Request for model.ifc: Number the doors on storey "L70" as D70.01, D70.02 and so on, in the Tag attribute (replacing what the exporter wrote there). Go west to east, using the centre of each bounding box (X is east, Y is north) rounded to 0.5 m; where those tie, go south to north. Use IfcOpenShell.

First a look at what the model holds.

```python
import ifcopenshell
import ifcopenshell.util.element
import ifcopenshell.util.placement

model = ifcopenshell.open("model.ifc")
print(model.schema)
storey = next(s for s in model.by_type("IfcBuildingStorey") if s.Name == "L70")
doors = [e for e in ifcopenshell.util.element.get_decomposition(storey) if e.is_a("IfcDoor")]
for e in sorted(doors, key=lambda e: e.id()):
    origin = ifcopenshell.util.placement.get_local_placement(e.ObjectPlacement)[:3, 3]
    print(e.id(), e.Tag, e.Name, origin.round(2) + 0.0, sep=" | ")
```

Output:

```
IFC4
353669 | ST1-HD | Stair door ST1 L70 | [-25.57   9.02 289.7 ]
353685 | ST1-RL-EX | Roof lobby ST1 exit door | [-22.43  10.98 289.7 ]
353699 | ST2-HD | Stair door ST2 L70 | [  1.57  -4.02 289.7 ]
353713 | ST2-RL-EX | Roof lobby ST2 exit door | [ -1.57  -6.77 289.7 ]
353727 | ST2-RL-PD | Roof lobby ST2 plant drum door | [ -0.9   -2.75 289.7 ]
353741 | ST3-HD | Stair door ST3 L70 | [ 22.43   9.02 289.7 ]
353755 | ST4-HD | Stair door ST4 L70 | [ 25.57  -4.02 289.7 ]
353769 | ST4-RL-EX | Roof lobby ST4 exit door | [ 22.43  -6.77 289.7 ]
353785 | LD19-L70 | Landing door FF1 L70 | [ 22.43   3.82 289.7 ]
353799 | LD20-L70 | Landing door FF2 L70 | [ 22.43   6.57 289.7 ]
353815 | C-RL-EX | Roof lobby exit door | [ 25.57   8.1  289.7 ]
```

```python
import ifcopenshell
import ifcopenshell.geom
import ifcopenshell.util.element
import ifcopenshell.util.shape

model = ifcopenshell.open("model.ifc")
settings = ifcopenshell.geom.settings()
settings.set("use-world-coords", True)


def centre(element):
    shape = ifcopenshell.geom.create_shape(settings, element)
    return ifcopenshell.util.shape.get_bbox_centroid(shape.geometry)


storey = next(s for s in model.by_type("IfcBuildingStorey") if s.Name == "L70")
doors = [e for e in ifcopenshell.util.element.get_decomposition(storey) if e.is_a("IfcDoor")]

# Insertion points can sit at a corner or the storey origin, so sort by the geometry (in metres).
centres = {e: centre(e) for e in doors}
doors.sort(key=lambda e: (round(centres[e][0] / 0.5), centres[e][1]))

for i, e in enumerate(doors, start=1):
    number = f"D70.{i:02d}"
    e.Tag = number
    print(e.id(), number)

model.write("model_v2.ifc")
```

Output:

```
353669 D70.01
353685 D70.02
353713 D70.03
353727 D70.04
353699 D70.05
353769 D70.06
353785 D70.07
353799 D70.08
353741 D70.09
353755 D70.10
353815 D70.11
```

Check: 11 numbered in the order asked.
